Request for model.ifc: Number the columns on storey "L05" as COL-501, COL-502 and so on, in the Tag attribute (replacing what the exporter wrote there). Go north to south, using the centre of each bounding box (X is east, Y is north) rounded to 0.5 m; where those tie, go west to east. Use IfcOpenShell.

First a look at what the model holds.

```python
import ifcopenshell
import ifcopenshell.util.element
import ifcopenshell.util.placement

model = ifcopenshell.open("model.ifc")
print(model.schema)
storey = next(s for s in model.by_type("IfcBuildingStorey") if s.Name == "L05")
columns = [e for e in ifcopenshell.util.element.get_decomposition(storey) if e.is_a("IfcColumn")]
for e in sorted(columns, key=lambda e: e.id()):
    origin = ifcopenshell.util.placement.get_local_placement(e.ObjectPlacement)[:3, 3]
    print(e.id(), e.Tag, e.Name, origin.round(2) + 0.0, sep=" | ")
```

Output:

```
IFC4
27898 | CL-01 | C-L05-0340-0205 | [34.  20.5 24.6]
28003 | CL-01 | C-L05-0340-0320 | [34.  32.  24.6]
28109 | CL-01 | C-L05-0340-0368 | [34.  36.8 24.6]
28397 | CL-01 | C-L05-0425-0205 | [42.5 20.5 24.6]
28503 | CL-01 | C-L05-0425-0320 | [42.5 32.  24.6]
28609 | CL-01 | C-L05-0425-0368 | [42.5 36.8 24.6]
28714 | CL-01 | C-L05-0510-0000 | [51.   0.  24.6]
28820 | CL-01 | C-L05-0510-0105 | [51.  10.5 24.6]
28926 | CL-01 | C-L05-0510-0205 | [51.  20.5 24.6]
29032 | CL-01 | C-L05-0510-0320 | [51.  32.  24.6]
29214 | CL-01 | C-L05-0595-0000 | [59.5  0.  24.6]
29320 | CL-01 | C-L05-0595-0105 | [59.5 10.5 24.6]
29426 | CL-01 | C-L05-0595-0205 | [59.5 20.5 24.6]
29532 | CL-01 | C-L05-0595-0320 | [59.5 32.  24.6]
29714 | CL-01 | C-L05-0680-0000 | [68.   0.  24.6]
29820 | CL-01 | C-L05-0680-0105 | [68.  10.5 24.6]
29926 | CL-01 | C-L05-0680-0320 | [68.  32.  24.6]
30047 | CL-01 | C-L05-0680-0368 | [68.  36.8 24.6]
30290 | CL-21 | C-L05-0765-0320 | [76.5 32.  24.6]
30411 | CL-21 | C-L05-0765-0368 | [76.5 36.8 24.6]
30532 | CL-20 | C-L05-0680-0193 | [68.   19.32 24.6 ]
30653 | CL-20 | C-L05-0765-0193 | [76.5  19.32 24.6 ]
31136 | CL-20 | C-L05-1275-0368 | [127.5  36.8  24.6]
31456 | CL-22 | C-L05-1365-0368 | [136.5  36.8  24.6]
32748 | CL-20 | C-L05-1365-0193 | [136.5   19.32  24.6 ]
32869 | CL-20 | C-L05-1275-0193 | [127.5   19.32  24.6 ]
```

```python
import ifcopenshell
import ifcopenshell.geom
import ifcopenshell.util.element
import ifcopenshell.util.shape

model = ifcopenshell.open("model.ifc")
settings = ifcopenshell.geom.settings()
settings.set("use-world-coords", True)


def centre(element):
    shape = ifcopenshell.geom.create_shape(settings, element)
    return ifcopenshell.util.shape.get_bbox_centroid(shape.geometry)


storey = next(s for s in model.by_type("IfcBuildingStorey") if s.Name == "L05")
columns = [e for e in ifcopenshell.util.element.get_decomposition(storey) if e.is_a("IfcColumn")]

# Insertion points can sit at a corner or the storey origin, so sort by the geometry (in metres).
centres = {e: centre(e) for e in columns}
columns.sort(key=lambda e: (-round(centres[e][1] / 0.5), centres[e][0]))

for i, e in enumerate(columns, start=1):
    number = f"COL-5{i:02d}"
    e.Tag = number
    print(e.id(), number)

model.write("model_v2.ifc")
```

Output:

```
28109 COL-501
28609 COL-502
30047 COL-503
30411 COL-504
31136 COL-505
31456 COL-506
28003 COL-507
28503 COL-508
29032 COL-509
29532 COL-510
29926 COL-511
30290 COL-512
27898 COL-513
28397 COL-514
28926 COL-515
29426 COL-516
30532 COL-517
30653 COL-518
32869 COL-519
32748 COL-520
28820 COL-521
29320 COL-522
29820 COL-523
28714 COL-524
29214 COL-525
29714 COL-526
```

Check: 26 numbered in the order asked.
